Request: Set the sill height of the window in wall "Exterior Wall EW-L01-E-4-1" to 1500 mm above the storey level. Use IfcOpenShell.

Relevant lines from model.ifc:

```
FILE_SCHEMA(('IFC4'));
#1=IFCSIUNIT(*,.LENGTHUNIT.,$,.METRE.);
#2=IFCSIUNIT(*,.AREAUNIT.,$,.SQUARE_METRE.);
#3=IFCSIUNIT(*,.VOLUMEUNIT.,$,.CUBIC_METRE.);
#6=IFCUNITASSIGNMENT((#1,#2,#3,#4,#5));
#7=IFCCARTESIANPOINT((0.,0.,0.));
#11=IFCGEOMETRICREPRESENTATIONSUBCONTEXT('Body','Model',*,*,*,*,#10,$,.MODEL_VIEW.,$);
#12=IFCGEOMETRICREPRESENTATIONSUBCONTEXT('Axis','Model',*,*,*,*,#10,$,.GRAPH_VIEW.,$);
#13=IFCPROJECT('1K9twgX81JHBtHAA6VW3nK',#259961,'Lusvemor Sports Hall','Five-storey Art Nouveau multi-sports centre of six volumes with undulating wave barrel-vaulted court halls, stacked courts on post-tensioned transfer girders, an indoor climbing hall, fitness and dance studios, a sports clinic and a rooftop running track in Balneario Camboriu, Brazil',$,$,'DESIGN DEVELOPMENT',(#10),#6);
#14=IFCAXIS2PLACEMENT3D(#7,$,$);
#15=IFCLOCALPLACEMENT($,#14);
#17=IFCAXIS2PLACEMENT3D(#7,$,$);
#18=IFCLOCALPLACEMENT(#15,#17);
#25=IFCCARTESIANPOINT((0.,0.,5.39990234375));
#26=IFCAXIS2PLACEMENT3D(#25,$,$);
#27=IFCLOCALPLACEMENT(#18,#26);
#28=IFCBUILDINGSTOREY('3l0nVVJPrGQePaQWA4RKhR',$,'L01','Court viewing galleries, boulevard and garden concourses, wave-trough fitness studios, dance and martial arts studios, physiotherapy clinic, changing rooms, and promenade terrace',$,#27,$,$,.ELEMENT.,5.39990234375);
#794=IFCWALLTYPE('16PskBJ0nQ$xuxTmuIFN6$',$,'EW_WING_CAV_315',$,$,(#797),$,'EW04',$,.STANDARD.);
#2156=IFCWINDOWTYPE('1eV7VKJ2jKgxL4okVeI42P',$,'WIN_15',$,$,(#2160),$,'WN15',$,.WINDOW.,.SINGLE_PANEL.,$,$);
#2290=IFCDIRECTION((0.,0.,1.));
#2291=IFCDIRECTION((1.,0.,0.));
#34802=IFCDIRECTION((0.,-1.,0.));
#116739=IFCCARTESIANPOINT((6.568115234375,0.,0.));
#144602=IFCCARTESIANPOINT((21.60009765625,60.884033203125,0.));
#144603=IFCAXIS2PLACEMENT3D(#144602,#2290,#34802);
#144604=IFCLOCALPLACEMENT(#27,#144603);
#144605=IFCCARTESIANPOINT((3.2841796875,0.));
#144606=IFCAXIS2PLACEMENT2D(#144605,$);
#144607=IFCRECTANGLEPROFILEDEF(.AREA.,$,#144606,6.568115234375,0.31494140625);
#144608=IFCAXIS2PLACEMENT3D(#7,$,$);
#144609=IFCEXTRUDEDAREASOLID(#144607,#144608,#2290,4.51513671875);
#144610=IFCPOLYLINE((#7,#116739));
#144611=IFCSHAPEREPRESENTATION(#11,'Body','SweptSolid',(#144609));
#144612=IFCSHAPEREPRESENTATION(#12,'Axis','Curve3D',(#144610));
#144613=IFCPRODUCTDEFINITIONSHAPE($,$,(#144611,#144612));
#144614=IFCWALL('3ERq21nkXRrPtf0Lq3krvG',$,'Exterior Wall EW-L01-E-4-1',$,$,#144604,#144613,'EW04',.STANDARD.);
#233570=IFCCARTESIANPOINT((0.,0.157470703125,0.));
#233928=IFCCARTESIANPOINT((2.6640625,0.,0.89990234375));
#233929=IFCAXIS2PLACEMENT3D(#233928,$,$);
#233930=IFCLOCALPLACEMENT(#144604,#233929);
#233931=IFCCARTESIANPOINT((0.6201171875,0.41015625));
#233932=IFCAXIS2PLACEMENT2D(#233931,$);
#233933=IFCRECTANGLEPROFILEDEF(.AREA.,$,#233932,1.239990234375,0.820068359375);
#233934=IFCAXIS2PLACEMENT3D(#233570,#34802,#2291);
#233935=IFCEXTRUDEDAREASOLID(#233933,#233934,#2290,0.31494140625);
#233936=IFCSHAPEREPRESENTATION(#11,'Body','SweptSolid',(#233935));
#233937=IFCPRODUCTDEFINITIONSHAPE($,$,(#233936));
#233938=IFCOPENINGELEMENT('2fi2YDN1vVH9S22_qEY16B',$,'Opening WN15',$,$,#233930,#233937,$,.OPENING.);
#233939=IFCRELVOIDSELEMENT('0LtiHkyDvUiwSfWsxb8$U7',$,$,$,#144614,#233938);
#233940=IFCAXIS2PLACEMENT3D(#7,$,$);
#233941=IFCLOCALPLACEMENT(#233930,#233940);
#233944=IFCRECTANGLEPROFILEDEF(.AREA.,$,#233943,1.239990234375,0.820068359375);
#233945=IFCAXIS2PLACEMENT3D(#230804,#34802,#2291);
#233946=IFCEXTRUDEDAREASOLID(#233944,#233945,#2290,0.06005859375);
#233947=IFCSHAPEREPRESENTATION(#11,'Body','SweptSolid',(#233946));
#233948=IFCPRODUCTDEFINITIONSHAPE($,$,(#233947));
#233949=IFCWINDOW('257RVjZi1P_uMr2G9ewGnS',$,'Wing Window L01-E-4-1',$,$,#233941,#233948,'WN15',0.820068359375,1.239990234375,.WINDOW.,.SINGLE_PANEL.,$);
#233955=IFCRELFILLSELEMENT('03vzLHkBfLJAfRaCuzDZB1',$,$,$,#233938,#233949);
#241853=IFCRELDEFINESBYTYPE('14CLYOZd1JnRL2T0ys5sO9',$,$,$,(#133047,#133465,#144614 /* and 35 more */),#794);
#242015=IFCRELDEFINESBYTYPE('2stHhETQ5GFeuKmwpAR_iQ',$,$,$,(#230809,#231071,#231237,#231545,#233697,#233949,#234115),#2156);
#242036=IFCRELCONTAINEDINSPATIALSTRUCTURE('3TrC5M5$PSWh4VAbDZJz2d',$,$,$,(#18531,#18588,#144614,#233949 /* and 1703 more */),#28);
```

```python
import numpy as np
import ifcopenshell
import ifcopenshell.api.geometry
import ifcopenshell.geom
import ifcopenshell.util.element
import ifcopenshell.util.placement
import ifcopenshell.util.shape
import ifcopenshell.util.unit

model = ifcopenshell.open("model.ifc")
unit_scale = ifcopenshell.util.unit.calculate_unit_scale(model)

window = model.by_id(233949)
opening = window.FillsVoids[0].RelatingOpeningElement
storey = ifcopenshell.util.element.get_container(window, ifc_class="IfcBuildingStorey")
level = ifcopenshell.util.placement.get_local_placement(storey.ObjectPlacement)[2, 3]

# The opening's origin need not be at the sill, so measure its lowest point.
shape = ifcopenshell.geom.create_shape(ifcopenshell.geom.settings(), opening)
bottom = ifcopenshell.util.shape.get_shape_bottom_elevation(shape, shape.geometry) / unit_scale
dz = level + 1.5 - bottom

shift = np.array([0.0, 0.0, dz])
# The window is placed relative to its opening, so it follows when the opening moves.
matrix = ifcopenshell.util.placement.get_local_placement(opening.ObjectPlacement)
matrix[:3, 3] += shift
ifcopenshell.api.geometry.edit_object_placement(
    model, product=opening, matrix=matrix, is_si=False, should_transform_children=True
)

print(f"moved by {dz * unit_scale:+.3f} m")

model.write("model_updated.ifc")
```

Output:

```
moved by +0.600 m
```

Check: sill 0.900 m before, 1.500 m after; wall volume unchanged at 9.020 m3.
